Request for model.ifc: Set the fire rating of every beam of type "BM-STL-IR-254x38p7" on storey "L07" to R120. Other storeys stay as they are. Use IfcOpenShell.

First a look at what the model holds.

```python
import ifcopenshell
import ifcopenshell.util.element

model = ifcopenshell.open("model.ifc")
print(model.schema)
storey = next(s for s in model.by_type("IfcBuildingStorey") if s.Name == "L07")
beams = [e for e in ifcopenshell.util.element.get_decomposition(storey) if e.is_a("IfcBeam")]
seen = {}
for e in beams:
    element_type = ifcopenshell.util.element.get_type(e)
    key = (element_type.Name if element_type != e and element_type else None, ifcopenshell.util.element.get_pset(e, "Pset_BeamCommon", "FireRating"))
    seen[key] = seen.get(key, 0) + 1
for (name, value), count in sorted(seen.items(), key=str):
    print(count, "x", name, "|", value)
```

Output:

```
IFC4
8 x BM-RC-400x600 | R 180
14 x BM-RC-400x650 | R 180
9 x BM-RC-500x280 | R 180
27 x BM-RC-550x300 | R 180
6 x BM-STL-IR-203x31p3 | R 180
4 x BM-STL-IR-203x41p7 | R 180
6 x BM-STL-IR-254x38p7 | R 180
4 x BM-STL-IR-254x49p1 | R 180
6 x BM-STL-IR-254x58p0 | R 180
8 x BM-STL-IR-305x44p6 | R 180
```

```python
import ifcopenshell
import ifcopenshell.api.pset
import ifcopenshell.util.element

model = ifcopenshell.open("model.ifc")

storey = next(s for s in model.by_type("IfcBuildingStorey") if s.Name == "L07")
beams = [e for e in ifcopenshell.util.element.get_decomposition(storey) if e.is_a("IfcBeam")]

count = 0
for e in beams:
    element_type = ifcopenshell.util.element.get_type(e)
    if element_type in (None, e) or element_type.Name != "BM-STL-IR-254x38p7":
        continue
    # add_pset returns the element's existing set when there is one.
    pset = ifcopenshell.api.pset.add_pset(model, product=e, name="Pset_BeamCommon")
    ifcopenshell.api.pset.edit_pset(model, pset=pset, properties={"FireRating": "R120"})
    count += 1

print(count, "beams updated")

model.write("model_edited.ifc")
```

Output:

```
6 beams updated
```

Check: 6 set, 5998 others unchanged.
